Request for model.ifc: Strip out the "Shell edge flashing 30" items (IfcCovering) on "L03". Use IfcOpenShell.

First a look at what the model holds.

```python
import ifcopenshell
import ifcopenshell.util.element

model = ifcopenshell.open("model.ifc")
print(model.schema)
storey = next(s for s in model.by_type("IfcBuildingStorey") if s.Name == "L03")
coverings = [e for e in ifcopenshell.util.element.get_decomposition(storey) if e.is_a("IfcCovering")]
seen = {}
for e in coverings:
    element_type = ifcopenshell.util.element.get_type(e)
    name = element_type.Name if element_type not in (None, e) else None
    seen[name] = seen.get(name, 0) + 1
for name, count in sorted(seen.items(), key=str):
    print(count, "x", name)
```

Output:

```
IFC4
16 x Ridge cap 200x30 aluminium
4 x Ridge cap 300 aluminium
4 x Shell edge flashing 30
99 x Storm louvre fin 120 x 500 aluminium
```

```python
import ifcopenshell
import ifcopenshell.api.root
import ifcopenshell.util.element

model = ifcopenshell.open("model.ifc")

storey = next(s for s in model.by_type("IfcBuildingStorey") if s.Name == "L03")
coverings = [e for e in ifcopenshell.util.element.get_decomposition(storey) if e.is_a("IfcCovering")]
targets = [e for e in coverings if (t := ifcopenshell.util.element.get_type(e)) not in (None, e) and t.Name == "Shell edge flashing 30"]

for e in targets:
    ifcopenshell.api.root.remove_product(model, product=e)
print(len(targets), "removed")

model.write("model_rev.ifc")
```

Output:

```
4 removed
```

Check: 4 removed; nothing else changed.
